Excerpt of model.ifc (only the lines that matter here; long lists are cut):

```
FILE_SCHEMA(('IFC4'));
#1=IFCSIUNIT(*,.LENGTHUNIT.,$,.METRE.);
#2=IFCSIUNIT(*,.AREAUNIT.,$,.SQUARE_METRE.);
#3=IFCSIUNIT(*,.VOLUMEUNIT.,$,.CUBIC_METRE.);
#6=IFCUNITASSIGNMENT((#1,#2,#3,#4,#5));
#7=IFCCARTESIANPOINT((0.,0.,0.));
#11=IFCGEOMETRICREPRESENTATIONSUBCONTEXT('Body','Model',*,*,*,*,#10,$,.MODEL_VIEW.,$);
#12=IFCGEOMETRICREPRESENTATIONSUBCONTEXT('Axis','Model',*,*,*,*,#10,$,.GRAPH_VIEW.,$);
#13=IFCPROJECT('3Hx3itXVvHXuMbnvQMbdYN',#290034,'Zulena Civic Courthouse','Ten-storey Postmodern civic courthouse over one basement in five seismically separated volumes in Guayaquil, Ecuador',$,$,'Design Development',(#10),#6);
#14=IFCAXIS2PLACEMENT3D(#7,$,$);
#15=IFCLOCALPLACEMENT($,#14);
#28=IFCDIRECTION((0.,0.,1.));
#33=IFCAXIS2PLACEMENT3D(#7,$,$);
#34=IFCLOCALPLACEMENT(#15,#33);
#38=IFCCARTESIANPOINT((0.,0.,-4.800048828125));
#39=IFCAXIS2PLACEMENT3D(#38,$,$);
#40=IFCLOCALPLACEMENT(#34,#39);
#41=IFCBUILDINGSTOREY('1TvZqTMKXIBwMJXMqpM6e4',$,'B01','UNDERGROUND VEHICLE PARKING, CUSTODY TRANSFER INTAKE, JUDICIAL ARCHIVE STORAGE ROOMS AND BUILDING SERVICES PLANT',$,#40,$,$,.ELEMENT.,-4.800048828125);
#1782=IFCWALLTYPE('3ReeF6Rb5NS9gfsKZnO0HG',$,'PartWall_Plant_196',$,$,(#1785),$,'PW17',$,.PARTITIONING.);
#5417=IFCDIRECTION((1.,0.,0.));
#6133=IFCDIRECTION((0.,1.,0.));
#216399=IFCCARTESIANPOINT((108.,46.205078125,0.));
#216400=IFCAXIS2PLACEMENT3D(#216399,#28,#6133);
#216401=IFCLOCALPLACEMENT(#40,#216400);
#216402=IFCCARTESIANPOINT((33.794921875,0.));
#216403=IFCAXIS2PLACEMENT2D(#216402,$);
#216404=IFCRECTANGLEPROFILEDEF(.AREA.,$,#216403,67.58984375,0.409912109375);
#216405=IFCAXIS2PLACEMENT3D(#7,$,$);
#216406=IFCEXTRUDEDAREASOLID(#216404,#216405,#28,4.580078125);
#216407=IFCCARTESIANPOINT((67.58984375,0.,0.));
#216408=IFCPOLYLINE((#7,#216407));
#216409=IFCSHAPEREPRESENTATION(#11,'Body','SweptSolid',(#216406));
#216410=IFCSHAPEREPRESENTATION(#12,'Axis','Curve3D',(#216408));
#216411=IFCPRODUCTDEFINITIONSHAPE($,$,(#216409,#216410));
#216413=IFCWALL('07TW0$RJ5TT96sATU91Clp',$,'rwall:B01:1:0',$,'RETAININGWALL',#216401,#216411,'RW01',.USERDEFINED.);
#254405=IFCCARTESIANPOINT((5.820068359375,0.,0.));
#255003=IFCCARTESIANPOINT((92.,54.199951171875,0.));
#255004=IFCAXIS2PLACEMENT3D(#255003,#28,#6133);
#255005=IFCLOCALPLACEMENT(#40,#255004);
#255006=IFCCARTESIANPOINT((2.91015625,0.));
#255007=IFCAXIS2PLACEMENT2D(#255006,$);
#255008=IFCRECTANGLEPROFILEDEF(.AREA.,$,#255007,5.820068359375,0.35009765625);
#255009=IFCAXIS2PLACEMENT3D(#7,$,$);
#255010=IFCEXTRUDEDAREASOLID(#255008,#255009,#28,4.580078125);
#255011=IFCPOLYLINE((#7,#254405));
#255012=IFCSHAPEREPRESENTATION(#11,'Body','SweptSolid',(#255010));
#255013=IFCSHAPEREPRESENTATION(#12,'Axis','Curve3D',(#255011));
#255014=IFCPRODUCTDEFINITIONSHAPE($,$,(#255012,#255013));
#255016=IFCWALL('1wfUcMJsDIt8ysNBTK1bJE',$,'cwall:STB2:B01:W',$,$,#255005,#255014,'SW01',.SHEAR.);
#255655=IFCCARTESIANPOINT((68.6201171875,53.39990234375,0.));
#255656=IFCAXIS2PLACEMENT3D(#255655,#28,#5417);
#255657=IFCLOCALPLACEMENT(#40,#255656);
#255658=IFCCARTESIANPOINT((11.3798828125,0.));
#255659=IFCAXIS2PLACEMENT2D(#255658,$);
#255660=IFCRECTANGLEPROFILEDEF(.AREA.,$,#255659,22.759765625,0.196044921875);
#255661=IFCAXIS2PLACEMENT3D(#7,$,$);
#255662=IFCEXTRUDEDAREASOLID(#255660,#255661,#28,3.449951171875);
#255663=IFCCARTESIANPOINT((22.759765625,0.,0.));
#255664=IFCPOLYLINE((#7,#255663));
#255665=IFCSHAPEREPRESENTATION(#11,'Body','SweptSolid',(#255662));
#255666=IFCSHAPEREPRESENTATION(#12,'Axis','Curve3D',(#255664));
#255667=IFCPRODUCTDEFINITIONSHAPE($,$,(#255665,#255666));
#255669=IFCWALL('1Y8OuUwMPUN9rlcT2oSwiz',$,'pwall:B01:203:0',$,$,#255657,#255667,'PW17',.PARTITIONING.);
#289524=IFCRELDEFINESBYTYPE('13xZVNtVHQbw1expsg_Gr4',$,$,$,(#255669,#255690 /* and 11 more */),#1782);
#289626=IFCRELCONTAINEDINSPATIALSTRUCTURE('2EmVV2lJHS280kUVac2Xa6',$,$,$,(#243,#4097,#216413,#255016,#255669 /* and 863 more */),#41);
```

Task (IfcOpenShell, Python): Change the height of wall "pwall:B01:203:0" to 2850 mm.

```python
import ifcopenshell
import ifcopenshell.geom
import ifcopenshell.util.representation
import ifcopenshell.util.shape

model = ifcopenshell.open("model.ifc")
settings = ifcopenshell.geom.settings()


def volume(element):
    """Net volume in cubic metres, openings subtracted."""
    shape = ifcopenshell.geom.create_shape(settings, element)
    return ifcopenshell.util.shape.get_volume(shape.geometry)


wall = model.by_guid("1Y8OuUwMPUN9rlcT2oSwiz")
before = volume(wall)

body = ifcopenshell.util.representation.get_representation(wall, "Model", "Body")
solid = body.Items[0]
old_height = solid.Depth
solid.Depth = 2.85
after = volume(wall)

print(f"height {old_height:g} -> {solid.Depth:g}, volume {before:.3f} -> {after:.3f} m3")

model.write("model-out.ifc")
```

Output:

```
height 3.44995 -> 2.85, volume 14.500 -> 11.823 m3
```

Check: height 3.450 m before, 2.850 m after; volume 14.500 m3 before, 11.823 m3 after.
